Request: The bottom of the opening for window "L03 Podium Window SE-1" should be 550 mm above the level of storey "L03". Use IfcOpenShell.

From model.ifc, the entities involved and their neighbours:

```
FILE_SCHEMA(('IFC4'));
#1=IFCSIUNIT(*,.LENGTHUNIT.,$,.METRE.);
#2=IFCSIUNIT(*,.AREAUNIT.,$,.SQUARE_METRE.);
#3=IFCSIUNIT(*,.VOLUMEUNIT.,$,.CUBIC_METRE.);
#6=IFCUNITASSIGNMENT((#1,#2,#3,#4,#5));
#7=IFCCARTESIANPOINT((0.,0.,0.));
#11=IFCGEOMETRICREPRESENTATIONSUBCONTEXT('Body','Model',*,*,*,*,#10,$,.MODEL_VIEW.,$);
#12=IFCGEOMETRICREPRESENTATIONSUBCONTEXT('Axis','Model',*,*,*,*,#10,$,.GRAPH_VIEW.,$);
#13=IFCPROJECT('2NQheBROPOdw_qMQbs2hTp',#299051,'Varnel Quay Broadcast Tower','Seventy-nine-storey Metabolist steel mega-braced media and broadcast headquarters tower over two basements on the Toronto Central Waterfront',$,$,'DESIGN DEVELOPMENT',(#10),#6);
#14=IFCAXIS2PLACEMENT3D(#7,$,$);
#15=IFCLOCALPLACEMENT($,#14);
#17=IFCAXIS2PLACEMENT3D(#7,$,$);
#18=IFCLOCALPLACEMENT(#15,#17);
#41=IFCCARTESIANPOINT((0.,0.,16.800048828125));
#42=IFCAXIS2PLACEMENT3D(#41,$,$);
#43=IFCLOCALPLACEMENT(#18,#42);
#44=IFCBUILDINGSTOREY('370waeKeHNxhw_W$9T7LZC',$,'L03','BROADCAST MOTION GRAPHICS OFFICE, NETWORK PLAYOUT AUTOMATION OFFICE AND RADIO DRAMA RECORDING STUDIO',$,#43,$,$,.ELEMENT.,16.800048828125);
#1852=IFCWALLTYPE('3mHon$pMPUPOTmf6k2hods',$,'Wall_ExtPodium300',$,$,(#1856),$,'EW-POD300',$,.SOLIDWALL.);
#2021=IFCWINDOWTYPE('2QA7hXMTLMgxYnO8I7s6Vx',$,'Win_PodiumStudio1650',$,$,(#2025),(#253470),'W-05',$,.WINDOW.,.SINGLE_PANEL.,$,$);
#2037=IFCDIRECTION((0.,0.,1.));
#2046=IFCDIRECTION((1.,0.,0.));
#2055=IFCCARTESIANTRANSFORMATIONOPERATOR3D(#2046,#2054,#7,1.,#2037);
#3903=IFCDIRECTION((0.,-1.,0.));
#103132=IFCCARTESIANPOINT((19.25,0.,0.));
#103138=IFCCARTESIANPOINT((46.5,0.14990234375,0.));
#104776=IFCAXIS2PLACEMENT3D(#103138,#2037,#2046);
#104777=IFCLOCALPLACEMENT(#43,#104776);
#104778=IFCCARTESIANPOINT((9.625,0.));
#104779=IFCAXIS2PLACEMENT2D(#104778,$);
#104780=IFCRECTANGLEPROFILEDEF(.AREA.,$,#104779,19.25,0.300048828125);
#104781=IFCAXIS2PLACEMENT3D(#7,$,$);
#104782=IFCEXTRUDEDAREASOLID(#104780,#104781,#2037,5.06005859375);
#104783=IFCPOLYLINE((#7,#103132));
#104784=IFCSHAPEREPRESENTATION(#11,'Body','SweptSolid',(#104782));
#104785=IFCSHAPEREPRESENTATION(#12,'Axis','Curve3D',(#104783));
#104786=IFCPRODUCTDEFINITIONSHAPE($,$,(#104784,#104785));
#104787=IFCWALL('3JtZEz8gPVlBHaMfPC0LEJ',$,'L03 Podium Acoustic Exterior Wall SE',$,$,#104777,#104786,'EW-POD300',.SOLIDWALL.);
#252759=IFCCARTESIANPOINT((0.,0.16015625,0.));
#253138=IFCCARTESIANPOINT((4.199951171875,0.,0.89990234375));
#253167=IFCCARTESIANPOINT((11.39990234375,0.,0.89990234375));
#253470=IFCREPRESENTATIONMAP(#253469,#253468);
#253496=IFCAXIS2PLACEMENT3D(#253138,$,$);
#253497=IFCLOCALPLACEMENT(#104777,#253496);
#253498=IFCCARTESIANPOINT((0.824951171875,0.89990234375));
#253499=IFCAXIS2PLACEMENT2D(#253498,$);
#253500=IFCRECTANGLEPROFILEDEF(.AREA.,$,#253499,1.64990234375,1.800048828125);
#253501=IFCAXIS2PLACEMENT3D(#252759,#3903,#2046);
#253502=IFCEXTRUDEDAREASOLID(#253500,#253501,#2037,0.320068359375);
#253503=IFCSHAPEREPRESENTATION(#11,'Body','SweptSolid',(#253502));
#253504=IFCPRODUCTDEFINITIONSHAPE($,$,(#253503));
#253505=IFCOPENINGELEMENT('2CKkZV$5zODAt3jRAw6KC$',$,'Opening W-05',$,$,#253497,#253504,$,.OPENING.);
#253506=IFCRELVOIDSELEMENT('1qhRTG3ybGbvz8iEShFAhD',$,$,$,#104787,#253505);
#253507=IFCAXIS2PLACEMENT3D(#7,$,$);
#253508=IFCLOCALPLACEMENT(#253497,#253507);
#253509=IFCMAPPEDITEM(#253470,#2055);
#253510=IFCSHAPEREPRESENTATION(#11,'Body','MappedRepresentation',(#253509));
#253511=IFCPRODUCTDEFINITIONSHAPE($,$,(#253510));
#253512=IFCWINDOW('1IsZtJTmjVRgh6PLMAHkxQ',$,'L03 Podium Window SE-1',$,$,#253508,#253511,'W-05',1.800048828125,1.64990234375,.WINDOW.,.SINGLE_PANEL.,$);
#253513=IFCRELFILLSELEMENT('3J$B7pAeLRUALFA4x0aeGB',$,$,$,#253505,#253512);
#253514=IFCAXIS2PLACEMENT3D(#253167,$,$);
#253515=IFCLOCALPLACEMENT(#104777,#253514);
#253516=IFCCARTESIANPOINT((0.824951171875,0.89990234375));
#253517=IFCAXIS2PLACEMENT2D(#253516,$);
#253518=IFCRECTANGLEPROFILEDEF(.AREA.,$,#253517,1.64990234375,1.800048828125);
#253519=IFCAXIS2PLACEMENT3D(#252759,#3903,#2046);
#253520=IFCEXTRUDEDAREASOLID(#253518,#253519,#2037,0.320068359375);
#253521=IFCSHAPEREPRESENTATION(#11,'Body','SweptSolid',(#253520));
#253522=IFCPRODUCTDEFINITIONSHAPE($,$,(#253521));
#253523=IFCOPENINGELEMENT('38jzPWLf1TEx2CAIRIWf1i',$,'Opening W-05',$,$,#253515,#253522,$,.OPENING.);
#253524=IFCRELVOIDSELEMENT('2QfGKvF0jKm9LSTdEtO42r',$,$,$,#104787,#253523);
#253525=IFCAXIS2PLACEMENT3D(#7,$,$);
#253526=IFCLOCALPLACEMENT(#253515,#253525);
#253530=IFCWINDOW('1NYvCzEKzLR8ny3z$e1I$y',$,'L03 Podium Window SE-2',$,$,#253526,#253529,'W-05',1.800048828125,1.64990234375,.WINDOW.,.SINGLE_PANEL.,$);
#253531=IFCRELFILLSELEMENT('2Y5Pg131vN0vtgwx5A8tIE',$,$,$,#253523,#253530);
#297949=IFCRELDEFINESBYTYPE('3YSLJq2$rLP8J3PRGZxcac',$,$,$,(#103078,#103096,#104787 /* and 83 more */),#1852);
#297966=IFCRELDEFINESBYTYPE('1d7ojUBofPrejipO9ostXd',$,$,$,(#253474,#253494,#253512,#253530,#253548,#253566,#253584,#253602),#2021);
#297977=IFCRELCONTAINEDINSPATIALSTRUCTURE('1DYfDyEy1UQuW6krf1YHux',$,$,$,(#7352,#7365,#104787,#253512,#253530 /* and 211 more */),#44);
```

```python
import numpy as np
import ifcopenshell
import ifcopenshell.api.geometry
import ifcopenshell.geom
import ifcopenshell.util.element
import ifcopenshell.util.placement
import ifcopenshell.util.shape
import ifcopenshell.util.unit

model = ifcopenshell.open("model.ifc")
unit_scale = ifcopenshell.util.unit.calculate_unit_scale(model)

window = model.by_guid("1IsZtJTmjVRgh6PLMAHkxQ")
opening = window.FillsVoids[0].RelatingOpeningElement
storey = ifcopenshell.util.element.get_container(window, ifc_class="IfcBuildingStorey")
level = ifcopenshell.util.placement.get_local_placement(storey.ObjectPlacement)[2, 3]

# The opening's origin need not be at the sill, so measure its lowest point.
shape = ifcopenshell.geom.create_shape(ifcopenshell.geom.settings(), opening)
bottom = ifcopenshell.util.shape.get_shape_bottom_elevation(shape, shape.geometry) / unit_scale
dz = level + 0.55 / unit_scale - bottom

shift = np.array([0.0, 0.0, dz])
# The window is placed relative to its opening, so it follows when the opening moves.
matrix = ifcopenshell.util.placement.get_local_placement(opening.ObjectPlacement)
matrix[:3, 3] += shift
ifcopenshell.api.geometry.edit_object_placement(
    model, product=opening, matrix=matrix, is_si=False, should_transform_children=True
)

print(f"moved by {dz * unit_scale:+.3f} m")

model.write("model_updated.ifc")
```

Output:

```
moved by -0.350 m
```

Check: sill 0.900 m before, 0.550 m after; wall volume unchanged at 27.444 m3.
